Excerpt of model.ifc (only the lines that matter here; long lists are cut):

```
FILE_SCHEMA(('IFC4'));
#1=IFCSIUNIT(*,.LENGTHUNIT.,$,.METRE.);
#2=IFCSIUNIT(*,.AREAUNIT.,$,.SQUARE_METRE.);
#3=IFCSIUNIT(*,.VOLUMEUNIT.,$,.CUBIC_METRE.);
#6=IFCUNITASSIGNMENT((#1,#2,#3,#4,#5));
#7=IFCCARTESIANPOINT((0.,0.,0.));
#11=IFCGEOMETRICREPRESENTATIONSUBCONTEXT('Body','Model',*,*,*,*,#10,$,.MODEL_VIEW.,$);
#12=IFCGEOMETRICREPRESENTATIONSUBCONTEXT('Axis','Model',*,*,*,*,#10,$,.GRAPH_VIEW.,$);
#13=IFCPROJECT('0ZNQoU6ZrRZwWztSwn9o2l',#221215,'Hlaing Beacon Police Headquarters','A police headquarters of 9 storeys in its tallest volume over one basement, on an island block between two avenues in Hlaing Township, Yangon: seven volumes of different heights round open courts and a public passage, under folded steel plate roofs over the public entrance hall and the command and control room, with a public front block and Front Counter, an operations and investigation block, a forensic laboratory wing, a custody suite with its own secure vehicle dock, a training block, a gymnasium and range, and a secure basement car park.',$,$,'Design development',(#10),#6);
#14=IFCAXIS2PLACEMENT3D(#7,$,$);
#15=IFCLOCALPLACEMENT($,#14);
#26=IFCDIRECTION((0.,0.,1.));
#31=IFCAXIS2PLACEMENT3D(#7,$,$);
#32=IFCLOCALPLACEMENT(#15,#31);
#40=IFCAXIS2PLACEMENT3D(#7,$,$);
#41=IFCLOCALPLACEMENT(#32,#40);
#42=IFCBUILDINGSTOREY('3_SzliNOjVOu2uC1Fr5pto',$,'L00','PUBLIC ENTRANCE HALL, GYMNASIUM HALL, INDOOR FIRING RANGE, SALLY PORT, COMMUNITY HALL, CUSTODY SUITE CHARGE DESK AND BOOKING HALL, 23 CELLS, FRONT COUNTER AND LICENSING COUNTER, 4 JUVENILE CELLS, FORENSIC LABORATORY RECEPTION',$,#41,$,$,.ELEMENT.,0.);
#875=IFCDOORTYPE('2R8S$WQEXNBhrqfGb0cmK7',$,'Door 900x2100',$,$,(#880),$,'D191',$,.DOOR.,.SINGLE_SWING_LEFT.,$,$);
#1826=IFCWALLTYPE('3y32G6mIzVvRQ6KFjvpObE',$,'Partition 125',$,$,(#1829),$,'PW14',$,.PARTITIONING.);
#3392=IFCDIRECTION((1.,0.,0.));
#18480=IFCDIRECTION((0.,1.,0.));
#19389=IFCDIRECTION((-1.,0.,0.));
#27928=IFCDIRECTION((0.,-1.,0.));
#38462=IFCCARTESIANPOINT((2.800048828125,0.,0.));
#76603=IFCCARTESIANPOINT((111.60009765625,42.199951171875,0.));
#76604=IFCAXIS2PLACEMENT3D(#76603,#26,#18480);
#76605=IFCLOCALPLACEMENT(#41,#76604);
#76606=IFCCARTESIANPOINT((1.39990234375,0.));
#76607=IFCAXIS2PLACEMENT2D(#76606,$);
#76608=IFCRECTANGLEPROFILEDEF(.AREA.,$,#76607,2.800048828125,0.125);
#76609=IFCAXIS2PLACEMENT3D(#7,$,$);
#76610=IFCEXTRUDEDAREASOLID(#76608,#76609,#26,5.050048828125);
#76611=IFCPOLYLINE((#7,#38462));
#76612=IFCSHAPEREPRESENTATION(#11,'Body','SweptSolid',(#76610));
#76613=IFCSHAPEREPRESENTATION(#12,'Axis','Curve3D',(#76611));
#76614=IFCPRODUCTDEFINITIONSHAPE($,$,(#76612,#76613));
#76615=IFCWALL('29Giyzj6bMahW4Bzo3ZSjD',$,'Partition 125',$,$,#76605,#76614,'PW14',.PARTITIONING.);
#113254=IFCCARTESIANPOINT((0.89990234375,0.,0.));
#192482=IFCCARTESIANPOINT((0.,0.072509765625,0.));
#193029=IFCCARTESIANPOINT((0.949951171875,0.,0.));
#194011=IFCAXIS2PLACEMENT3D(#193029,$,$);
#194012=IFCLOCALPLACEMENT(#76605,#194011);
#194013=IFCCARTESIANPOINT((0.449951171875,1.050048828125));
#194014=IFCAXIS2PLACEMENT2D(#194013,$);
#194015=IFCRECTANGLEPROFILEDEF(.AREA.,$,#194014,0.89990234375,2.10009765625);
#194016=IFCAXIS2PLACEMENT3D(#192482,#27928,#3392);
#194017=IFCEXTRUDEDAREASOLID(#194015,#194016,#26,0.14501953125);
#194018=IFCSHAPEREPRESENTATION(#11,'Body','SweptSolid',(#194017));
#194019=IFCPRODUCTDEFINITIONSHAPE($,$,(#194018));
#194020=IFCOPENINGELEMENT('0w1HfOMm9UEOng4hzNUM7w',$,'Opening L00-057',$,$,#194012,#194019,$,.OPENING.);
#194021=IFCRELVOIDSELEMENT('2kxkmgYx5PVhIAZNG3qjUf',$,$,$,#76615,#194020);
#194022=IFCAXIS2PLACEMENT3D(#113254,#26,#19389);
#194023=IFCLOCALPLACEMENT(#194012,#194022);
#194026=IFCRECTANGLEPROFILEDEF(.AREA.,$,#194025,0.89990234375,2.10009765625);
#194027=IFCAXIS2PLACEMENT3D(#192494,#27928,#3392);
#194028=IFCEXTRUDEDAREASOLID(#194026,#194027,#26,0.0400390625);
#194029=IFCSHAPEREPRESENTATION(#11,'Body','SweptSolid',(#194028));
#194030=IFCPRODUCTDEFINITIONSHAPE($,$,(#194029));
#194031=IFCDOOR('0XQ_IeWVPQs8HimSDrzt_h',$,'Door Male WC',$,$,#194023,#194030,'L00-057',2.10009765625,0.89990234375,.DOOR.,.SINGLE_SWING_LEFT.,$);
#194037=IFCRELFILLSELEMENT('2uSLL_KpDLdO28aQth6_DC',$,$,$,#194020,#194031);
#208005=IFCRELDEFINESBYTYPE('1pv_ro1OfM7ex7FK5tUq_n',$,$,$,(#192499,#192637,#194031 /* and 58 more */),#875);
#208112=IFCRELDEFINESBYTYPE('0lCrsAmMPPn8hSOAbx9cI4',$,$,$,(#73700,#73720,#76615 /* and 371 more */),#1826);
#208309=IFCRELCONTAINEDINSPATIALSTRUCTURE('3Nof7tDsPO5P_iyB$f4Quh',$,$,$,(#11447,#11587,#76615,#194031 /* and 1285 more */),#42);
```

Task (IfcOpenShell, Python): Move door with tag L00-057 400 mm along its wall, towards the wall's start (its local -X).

```python
import ifcopenshell
import ifcopenshell.api.geometry
import ifcopenshell.util.placement
import ifcopenshell.util.unit

model = ifcopenshell.open("model.ifc")
unit_scale = ifcopenshell.util.unit.calculate_unit_scale(model)

door = model.by_guid("0XQ_IeWVPQs8HimSDrzt_h")
opening = door.FillsVoids[0].RelatingOpeningElement
wall = opening.VoidsElements[0].RelatingBuildingElement

wall_matrix = ifcopenshell.util.placement.get_local_placement(wall.ObjectPlacement)
shift = wall_matrix[:3, 0] * -0.4 / unit_scale
before = ifcopenshell.util.placement.get_local_placement(door.ObjectPlacement)[:3, 3].copy()

# The door is placed relative to its opening, so it follows when the opening moves.
matrix = ifcopenshell.util.placement.get_local_placement(opening.ObjectPlacement)
matrix[:3, 3] += shift
ifcopenshell.api.geometry.edit_object_placement(
    model, product=opening, matrix=matrix, is_si=False, should_transform_children=True
)

after = ifcopenshell.util.placement.get_local_placement(door.ObjectPlacement)[:3, 3]
print("door moved by", (after - before).round(3) + 0.0)

model.write("model_rev.ifc")
```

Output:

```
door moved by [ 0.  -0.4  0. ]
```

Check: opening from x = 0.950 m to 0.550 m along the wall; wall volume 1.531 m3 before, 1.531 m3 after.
